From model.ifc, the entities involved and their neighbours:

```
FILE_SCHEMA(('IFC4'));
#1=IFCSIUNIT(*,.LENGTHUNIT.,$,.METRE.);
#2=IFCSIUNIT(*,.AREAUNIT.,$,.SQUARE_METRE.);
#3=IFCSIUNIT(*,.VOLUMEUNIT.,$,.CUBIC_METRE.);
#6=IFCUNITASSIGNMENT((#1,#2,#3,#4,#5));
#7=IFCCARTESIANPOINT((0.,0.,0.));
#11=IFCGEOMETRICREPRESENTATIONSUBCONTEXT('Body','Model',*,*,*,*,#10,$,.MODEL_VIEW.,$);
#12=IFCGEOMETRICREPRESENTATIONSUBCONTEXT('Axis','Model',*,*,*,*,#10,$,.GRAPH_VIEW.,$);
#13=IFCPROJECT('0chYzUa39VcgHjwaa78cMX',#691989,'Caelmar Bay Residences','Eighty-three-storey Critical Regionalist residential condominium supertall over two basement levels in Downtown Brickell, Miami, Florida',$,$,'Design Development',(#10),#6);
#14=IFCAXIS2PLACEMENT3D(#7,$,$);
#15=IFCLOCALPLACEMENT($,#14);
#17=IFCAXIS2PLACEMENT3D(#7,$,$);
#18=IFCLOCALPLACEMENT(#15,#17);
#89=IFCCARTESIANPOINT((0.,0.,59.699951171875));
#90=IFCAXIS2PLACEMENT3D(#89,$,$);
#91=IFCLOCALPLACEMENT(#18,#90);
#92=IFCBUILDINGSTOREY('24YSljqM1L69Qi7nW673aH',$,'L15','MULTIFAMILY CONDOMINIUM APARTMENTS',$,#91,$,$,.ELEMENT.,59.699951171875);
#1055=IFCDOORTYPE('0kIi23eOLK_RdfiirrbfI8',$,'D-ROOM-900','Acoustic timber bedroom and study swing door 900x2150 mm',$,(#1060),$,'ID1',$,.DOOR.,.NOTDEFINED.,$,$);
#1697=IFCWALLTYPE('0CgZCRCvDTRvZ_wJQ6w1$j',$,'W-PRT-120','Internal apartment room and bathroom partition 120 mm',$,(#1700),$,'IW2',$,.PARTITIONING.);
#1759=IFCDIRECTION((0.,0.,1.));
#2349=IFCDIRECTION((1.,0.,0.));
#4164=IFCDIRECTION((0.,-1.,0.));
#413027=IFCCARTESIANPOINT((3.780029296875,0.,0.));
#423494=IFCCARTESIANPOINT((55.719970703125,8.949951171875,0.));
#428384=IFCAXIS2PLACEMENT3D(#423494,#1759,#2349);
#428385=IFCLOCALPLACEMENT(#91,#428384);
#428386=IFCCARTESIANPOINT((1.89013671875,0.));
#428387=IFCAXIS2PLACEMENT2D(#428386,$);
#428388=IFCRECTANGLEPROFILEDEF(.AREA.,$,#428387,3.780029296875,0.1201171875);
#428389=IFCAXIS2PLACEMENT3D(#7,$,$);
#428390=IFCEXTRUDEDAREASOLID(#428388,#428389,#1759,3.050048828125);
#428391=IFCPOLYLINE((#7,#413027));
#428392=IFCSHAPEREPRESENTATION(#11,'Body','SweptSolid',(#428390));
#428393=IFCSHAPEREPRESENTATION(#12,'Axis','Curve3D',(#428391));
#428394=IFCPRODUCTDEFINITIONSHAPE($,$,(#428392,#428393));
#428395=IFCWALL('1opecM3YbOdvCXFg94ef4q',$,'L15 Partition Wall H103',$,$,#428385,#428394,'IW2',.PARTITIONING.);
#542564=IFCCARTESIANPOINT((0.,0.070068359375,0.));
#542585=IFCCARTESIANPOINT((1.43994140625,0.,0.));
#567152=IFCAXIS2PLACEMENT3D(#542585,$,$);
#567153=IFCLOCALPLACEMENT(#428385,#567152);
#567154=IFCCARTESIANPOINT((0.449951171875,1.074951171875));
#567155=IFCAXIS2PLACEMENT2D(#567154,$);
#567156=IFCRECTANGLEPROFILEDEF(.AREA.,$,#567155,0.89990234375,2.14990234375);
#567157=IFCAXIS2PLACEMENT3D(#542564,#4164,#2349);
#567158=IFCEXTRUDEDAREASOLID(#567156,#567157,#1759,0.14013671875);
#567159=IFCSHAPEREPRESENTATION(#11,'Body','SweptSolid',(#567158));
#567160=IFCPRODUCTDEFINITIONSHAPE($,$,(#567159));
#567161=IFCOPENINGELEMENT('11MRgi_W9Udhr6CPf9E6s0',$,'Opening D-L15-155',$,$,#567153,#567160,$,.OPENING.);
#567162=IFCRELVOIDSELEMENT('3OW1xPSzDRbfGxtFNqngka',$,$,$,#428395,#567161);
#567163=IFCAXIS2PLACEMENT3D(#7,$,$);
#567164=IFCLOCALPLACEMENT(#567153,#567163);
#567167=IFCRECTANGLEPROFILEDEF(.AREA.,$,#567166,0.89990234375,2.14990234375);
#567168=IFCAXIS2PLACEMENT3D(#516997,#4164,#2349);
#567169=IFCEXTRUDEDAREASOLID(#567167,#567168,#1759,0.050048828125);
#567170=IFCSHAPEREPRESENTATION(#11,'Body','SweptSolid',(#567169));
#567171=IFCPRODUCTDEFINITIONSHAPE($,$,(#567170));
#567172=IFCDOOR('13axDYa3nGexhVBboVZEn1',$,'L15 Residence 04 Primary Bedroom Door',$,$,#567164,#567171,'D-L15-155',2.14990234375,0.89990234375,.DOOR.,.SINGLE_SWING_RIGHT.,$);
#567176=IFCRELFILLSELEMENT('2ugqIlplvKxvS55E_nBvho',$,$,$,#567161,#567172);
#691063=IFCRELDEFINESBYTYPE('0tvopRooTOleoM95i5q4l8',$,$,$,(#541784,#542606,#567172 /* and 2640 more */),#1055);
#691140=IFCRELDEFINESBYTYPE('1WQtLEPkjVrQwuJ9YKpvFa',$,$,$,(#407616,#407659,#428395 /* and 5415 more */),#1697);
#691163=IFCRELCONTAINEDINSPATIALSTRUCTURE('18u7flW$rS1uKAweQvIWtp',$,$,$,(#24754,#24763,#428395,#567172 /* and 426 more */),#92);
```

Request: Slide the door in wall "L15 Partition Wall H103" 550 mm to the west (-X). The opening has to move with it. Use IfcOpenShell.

```python
import ifcopenshell
import ifcopenshell.api.geometry
import ifcopenshell.util.placement

model = ifcopenshell.open("model.ifc")

door = model.by_guid("13axDYa3nGexhVBboVZEn1")
opening = door.FillsVoids[0].RelatingOpeningElement
wall = opening.VoidsElements[0].RelatingBuildingElement

wall_matrix = ifcopenshell.util.placement.get_local_placement(wall.ObjectPlacement)
shift = wall_matrix[:3, 0] * -0.55
before = ifcopenshell.util.placement.get_local_placement(door.ObjectPlacement)[:3, 3].copy()

# The door is placed relative to its opening, so it follows when the opening moves.
matrix = ifcopenshell.util.placement.get_local_placement(opening.ObjectPlacement)
matrix[:3, 3] += shift
ifcopenshell.api.geometry.edit_object_placement(
    model, product=opening, matrix=matrix, is_si=False, should_transform_children=True
)

after = ifcopenshell.util.placement.get_local_placement(door.ObjectPlacement)[:3, 3]
print("door moved by", (after - before).round(3) + 0.0)

model.write("model_updated.ifc")
```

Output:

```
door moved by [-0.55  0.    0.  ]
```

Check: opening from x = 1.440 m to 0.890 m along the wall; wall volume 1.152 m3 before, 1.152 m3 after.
